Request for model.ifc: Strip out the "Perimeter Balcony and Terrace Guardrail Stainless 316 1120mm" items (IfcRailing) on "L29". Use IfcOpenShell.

First a look at what the model holds.

```python
import ifcopenshell
import ifcopenshell.util.element

model = ifcopenshell.open("model.ifc")
print(model.schema)
storey = next(s for s in model.by_type("IfcBuildingStorey") if s.Name == "L29")
railings = [e for e in ifcopenshell.util.element.get_decomposition(storey) if e.is_a("IfcRailing")]
seen = {}
for e in railings:
    element_type = ifcopenshell.util.element.get_type(e)
    name = element_type.Name if element_type not in (None, e) else None
    seen[name] = seen.get(name, 0) + 1
for name, count in sorted(seen.items(), key=str):
    print(count, "x", name)
```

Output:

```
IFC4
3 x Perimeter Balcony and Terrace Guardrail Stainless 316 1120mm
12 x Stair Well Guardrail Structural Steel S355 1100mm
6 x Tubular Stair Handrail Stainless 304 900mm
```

```python
import ifcopenshell
import ifcopenshell.api.root
import ifcopenshell.util.element

model = ifcopenshell.open("model.ifc")

storey = next(s for s in model.by_type("IfcBuildingStorey") if s.Name == "L29")
railings = [e for e in ifcopenshell.util.element.get_decomposition(storey) if e.is_a("IfcRailing")]
targets = [e for e in railings if (t := ifcopenshell.util.element.get_type(e)) not in (None, e) and t.Name == "Perimeter Balcony and Terrace Guardrail Stainless 316 1120mm"]

for e in targets:
    ifcopenshell.api.root.remove_product(model, product=e)
print(len(targets), "removed")

model.write("model_updated.ifc")
```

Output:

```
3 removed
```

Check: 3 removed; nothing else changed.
